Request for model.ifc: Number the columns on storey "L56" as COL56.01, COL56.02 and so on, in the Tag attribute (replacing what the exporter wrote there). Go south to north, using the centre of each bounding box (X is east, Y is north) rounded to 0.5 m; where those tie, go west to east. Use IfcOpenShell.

First a look at what the model holds.

```python
import ifcopenshell
import ifcopenshell.util.element
import ifcopenshell.util.placement

model = ifcopenshell.open("model.ifc")
print(model.schema)
storey = next(s for s in model.by_type("IfcBuildingStorey") if s.Name == "L56")
columns = [e for e in ifcopenshell.util.element.get_decomposition(storey) if e.is_a("IfcColumn")]
for e in sorted(columns, key=lambda e: e.id()):
    origin = ifcopenshell.util.placement.get_local_placement(e.ObjectPlacement)[:3, 3]
    print(e.id(), e.Tag, e.Name, origin.round(2) + 0.0, sep=" | ")
```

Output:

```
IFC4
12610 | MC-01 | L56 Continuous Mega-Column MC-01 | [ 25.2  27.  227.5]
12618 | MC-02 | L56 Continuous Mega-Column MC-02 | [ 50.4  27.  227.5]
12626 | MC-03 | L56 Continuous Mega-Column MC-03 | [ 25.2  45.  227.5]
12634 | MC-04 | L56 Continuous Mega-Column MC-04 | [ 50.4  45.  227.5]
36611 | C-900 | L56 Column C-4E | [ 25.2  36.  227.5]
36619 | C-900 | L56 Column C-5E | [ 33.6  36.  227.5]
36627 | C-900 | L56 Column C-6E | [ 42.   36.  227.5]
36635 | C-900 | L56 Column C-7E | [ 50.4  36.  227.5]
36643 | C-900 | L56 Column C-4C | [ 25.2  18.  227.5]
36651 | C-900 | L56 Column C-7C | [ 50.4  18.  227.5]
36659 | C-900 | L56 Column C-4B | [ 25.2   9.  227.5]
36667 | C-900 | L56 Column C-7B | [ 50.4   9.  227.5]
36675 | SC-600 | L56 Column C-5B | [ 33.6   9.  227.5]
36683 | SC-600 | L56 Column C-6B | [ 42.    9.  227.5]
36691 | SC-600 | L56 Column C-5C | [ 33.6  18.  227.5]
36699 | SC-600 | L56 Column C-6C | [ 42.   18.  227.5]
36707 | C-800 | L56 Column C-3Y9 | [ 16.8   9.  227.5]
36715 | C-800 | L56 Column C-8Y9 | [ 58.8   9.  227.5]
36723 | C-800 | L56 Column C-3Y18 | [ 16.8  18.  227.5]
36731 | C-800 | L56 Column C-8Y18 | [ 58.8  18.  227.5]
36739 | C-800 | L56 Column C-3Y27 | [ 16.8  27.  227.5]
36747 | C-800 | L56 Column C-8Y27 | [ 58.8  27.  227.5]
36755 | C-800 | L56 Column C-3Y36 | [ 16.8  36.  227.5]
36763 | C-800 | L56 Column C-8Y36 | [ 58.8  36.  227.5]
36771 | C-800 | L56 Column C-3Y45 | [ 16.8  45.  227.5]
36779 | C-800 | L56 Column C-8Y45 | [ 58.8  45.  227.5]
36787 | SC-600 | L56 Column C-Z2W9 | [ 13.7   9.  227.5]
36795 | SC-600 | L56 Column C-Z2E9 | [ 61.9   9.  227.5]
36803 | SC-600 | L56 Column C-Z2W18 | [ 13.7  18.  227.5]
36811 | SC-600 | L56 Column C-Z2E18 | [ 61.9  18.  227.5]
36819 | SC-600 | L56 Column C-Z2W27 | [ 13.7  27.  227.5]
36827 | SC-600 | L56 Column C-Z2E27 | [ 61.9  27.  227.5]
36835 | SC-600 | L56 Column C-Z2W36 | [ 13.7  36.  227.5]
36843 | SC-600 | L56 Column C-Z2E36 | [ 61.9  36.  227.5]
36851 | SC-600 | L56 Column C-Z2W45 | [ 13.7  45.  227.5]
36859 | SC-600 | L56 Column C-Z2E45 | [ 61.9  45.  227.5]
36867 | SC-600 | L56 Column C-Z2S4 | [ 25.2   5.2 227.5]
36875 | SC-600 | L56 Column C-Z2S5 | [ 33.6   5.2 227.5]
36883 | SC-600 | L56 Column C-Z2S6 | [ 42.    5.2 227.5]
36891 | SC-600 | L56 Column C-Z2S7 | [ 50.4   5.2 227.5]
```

```python
import ifcopenshell
import ifcopenshell.geom
import ifcopenshell.util.element
import ifcopenshell.util.shape

model = ifcopenshell.open("model.ifc")
settings = ifcopenshell.geom.settings()
settings.set("use-world-coords", True)


def centre(element):
    shape = ifcopenshell.geom.create_shape(settings, element)
    return ifcopenshell.util.shape.get_bbox_centroid(shape.geometry)


storey = next(s for s in model.by_type("IfcBuildingStorey") if s.Name == "L56")
columns = [e for e in ifcopenshell.util.element.get_decomposition(storey) if e.is_a("IfcColumn")]

# Insertion points can sit at a corner or the storey origin, so sort by the geometry (in metres).
centres = {e: centre(e) for e in columns}
columns.sort(key=lambda e: (round(centres[e][1] / 0.5), centres[e][0]))

for i, e in enumerate(columns, start=1):
    number = f"COL56.{i:02d}"
    e.Tag = number
    print(e.id(), number)

model.write("model_updated.ifc")
```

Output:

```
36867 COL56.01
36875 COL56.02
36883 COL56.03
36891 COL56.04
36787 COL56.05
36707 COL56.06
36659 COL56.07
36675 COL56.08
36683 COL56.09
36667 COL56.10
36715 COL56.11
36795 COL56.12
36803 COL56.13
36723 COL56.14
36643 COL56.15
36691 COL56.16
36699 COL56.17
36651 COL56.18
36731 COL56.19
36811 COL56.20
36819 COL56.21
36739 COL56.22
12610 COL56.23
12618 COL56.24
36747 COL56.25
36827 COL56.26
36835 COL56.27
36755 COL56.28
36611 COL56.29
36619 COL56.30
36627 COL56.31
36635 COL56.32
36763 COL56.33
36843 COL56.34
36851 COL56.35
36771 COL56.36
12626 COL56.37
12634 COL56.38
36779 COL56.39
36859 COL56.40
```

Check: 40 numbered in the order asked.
